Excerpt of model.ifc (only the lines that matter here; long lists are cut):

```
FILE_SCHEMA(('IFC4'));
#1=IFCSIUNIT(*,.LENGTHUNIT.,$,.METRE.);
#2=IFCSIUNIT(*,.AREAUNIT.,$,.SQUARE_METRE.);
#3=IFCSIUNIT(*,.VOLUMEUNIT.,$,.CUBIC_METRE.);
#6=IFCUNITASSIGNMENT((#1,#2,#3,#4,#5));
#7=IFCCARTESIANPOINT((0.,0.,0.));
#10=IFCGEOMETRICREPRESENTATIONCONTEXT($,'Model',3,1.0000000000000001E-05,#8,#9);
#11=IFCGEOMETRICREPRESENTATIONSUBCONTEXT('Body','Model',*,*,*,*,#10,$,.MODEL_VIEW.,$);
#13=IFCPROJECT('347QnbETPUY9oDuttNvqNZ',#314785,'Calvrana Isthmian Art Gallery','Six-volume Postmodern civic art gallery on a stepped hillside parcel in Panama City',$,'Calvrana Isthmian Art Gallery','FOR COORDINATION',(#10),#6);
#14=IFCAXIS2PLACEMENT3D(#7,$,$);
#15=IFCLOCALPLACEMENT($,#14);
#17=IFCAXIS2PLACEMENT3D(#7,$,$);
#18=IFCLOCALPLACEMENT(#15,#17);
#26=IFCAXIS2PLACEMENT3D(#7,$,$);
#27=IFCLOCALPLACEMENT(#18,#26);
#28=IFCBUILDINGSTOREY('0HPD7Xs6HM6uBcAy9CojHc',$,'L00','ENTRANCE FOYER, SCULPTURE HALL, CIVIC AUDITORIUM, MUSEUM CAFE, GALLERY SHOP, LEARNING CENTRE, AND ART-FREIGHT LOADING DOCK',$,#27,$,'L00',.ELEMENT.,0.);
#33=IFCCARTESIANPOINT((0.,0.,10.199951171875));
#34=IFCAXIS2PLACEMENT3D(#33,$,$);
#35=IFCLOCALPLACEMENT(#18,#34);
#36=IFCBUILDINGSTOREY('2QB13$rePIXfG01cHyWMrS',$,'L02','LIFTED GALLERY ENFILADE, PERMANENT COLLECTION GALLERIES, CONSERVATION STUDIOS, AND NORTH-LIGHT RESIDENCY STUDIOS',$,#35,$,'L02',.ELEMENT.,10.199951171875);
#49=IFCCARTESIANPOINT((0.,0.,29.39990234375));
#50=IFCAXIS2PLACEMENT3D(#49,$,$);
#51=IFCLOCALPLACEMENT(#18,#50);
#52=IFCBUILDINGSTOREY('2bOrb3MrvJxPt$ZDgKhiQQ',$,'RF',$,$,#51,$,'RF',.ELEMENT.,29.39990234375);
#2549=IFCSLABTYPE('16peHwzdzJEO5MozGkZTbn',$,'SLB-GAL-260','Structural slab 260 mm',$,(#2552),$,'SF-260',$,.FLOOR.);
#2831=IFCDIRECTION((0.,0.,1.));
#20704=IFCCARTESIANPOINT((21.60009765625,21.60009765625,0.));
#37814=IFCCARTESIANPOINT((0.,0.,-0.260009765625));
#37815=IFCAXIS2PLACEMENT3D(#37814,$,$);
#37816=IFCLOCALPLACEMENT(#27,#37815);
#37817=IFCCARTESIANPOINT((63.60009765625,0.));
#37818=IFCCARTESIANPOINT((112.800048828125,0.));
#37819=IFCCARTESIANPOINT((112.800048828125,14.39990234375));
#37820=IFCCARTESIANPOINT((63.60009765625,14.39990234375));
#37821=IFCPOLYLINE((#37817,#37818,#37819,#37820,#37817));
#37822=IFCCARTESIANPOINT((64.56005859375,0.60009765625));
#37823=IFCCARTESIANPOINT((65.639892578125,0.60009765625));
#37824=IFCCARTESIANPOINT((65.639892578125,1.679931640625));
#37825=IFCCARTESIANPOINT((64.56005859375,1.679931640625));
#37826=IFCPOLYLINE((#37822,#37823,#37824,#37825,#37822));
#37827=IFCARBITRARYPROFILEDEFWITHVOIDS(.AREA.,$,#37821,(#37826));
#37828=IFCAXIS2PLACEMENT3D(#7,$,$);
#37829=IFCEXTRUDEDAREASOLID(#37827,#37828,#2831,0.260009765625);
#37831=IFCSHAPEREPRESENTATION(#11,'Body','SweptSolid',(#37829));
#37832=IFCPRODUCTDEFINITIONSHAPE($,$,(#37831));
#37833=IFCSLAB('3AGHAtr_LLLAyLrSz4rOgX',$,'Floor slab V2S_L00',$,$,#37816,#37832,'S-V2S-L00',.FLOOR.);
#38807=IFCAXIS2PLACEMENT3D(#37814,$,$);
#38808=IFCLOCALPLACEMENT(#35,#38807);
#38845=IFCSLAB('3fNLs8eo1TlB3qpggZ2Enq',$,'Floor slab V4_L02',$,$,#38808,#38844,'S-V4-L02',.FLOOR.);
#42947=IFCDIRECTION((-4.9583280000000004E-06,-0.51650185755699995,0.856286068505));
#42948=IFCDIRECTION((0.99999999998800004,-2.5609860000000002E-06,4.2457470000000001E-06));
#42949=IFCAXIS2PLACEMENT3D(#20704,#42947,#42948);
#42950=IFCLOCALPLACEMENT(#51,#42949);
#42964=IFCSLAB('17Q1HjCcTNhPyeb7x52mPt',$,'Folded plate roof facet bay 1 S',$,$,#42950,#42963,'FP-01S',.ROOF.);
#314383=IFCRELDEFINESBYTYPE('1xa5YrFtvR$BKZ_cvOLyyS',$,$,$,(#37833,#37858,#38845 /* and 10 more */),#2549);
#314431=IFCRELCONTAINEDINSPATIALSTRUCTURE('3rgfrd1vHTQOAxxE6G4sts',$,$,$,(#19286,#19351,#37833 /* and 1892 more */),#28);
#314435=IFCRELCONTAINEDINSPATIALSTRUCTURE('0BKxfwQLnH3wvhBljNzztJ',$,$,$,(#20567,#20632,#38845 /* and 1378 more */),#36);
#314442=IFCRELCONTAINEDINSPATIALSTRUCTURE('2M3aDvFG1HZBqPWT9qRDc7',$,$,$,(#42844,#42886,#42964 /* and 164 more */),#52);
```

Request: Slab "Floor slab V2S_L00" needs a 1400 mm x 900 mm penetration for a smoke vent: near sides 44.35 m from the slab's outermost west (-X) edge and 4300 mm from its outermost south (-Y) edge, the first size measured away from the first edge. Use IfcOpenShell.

```python
import numpy as np
import ifcopenshell
import ifcopenshell.api.feature
import ifcopenshell.api.geometry
import ifcopenshell.api.root
import ifcopenshell.geom
import ifcopenshell.util.placement
import ifcopenshell.util.representation
import ifcopenshell.util.shape
import ifcopenshell.util.unit

model = ifcopenshell.open("model.ifc")
unit_scale = ifcopenshell.util.unit.calculate_unit_scale(model)
settings = ifcopenshell.geom.settings()


def volume(element):
    """Net volume in cubic metres, openings subtracted."""
    shape = ifcopenshell.geom.create_shape(settings, element)
    return ifcopenshell.util.shape.get_volume(shape.geometry)


slab = model.by_id(37833)
before = volume(slab)

# Extent in the slab's own axes, in metres. The edges named are its -X and -Y sides.
slab_shape = ifcopenshell.geom.create_shape(settings, slab)
vertices = ifcopenshell.util.shape.get_vertices(slab_shape.geometry)
x_min, y_min, bottom = vertices.min(axis=0)
top = vertices[:, 2].max()

opening = ifcopenshell.api.root.create_entity(model, ifc_class="IfcOpeningElement", name="Smoke vent opening", predefined_type="OPENING")
context = ifcopenshell.util.representation.get_context(model, "Model", "Body", "MODEL_VIEW")
width, depth = 1.4, 0.9
outline = [(0.0, 0.0), (width, 0.0), (width, depth), (0.0, depth), (0.0, 0.0)]
# Overshoot both faces by 50 mm so the cut is clean.
shape = ifcopenshell.api.geometry.add_slab_representation(
    model, context=context, depth=top - bottom + 0.1, polyline=outline
)
ifcopenshell.api.geometry.assign_representation(model, product=opening, representation=shape)

matrix = ifcopenshell.util.placement.get_local_placement(slab.ObjectPlacement)
matrix[:, 3] = matrix @ np.append(np.array([x_min + 44.35, y_min + 4.3, bottom - 0.05]) / unit_scale, 1.0)
ifcopenshell.api.geometry.edit_object_placement(model, product=opening, matrix=matrix, is_si=False)
ifcopenshell.api.feature.add_feature(model, feature=opening, element=slab)

after = volume(slab)

print(f"slab volume {before:.3f} -> {after:.3f} m3")

model.write("model_rev.ifc")
```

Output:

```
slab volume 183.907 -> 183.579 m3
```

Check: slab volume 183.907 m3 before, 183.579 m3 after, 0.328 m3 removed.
